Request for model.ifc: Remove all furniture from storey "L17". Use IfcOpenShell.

First a look at what the model holds.

```python
import ifcopenshell
import ifcopenshell.util.element

model = ifcopenshell.open("model.ifc")
print(model.schema)
storey = next(s for s in model.by_type("IfcBuildingStorey") if s.Name == "L17")
furniture = [e for e in ifcopenshell.util.element.get_decomposition(storey) if e.is_a("IfcFurnishingElement")]
seen = {}
for e in furniture:
    element_type = ifcopenshell.util.element.get_type(e)
    name = element_type.Name if element_type not in (None, e) else None
    seen[name] = seen.get(name, 0) + 1
for name, count in sorted(seen.items(), key=str):
    print(count, "x", name)
```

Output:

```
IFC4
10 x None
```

```python
import ifcopenshell
import ifcopenshell.api.root
import ifcopenshell.util.element

model = ifcopenshell.open("model.ifc")

storey = next(s for s in model.by_type("IfcBuildingStorey") if s.Name == "L17")
furniture = [e for e in ifcopenshell.util.element.get_decomposition(storey) if e.is_a("IfcFurnishingElement")]

for e in furniture:
    ifcopenshell.api.root.remove_product(model, product=e)
print(len(furniture), "removed")

model.write("model_v2.ifc")
```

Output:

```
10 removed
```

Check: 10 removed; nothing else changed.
